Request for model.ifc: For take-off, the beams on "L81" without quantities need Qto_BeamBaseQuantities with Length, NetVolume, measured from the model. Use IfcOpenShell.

First a look at what the model holds.

```python
import ifcopenshell
import ifcopenshell.util.element
import ifcopenshell.util.unit

model = ifcopenshell.open("model.ifc")
print(model.schema)
for unit_type in ("LENGTHUNIT", "AREAUNIT", "VOLUMEUNIT"):
    print(unit_type, ifcopenshell.util.unit.calculate_unit_scale(model, unit_type))
storey = next(s for s in model.by_type("IfcBuildingStorey") if s.Name == "L81")
beams = [e for e in ifcopenshell.util.element.get_decomposition(storey) if e.is_a("IfcBeam")]
for e in sorted(beams, key=lambda e: e.id()):
    print(e.id(), e.is_a(), e.Name, list(ifcopenshell.util.element.get_psets(e, qtos_only=True)), sep=" | ")
```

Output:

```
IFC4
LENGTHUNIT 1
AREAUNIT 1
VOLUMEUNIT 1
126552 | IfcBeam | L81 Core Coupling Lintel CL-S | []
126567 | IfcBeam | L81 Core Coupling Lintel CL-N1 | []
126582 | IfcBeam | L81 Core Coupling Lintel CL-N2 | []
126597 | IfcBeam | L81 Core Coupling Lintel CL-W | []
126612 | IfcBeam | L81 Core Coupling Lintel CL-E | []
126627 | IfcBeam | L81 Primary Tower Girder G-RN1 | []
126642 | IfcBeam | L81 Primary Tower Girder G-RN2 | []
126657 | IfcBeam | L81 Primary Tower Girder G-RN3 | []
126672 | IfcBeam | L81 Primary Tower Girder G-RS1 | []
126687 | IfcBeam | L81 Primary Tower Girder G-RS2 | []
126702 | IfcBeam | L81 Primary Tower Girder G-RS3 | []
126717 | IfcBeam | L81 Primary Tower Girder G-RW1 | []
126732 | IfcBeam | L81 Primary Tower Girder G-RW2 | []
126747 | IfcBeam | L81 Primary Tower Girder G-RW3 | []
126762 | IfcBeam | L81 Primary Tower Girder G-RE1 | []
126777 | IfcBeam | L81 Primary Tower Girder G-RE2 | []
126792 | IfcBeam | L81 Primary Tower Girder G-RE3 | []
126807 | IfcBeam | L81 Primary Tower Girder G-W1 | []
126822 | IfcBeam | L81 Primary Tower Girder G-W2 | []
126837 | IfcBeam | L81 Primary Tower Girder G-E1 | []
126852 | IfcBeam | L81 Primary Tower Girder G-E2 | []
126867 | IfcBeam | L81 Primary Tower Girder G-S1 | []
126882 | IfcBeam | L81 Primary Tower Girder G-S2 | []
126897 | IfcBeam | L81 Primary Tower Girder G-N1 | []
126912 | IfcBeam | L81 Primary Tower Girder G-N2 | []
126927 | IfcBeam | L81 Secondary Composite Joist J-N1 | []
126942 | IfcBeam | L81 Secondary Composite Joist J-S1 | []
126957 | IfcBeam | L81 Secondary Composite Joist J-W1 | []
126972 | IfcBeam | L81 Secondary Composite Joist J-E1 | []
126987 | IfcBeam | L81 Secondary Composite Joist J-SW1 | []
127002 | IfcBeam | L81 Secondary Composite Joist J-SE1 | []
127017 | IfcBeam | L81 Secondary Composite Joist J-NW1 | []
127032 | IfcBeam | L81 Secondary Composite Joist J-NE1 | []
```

```python
import ifcopenshell
import ifcopenshell.api.pset
import ifcopenshell.geom
import ifcopenshell.util.element
import ifcopenshell.util.shape
import ifcopenshell.util.unit

model = ifcopenshell.open("model.ifc")
unit_scale = ifcopenshell.util.unit.calculate_unit_scale(model)
volume_scale = ifcopenshell.util.unit.calculate_unit_scale(model, "VOLUMEUNIT")
settings = ifcopenshell.geom.settings()

storey = next(s for s in model.by_type("IfcBuildingStorey") if s.Name == "L81")
beams = [e for e in ifcopenshell.util.element.get_decomposition(storey) if e.is_a("IfcBeam")]

for e in sorted(beams, key=lambda e: e.id()):
    if ifcopenshell.util.element.get_psets(e, qtos_only=True, should_inherit=False):
        continue
    # Geometry comes back in metres, in the element's own axes.
    shape = ifcopenshell.geom.create_shape(settings, e)
    values = {
        "Length": ifcopenshell.util.shape.get_max_xyz(shape.geometry) / unit_scale,
        "NetVolume": ifcopenshell.util.shape.get_volume(shape.geometry) / volume_scale,
    }
    qto = ifcopenshell.api.pset.add_qto(model, product=e, name="Qto_BeamBaseQuantities")
    ifcopenshell.api.pset.edit_qto(model, qto=qto, properties=values)
    print(e.id(), {k: round(v, 3) for k, v in values.items()})

model.write("model_v2.ifc")
```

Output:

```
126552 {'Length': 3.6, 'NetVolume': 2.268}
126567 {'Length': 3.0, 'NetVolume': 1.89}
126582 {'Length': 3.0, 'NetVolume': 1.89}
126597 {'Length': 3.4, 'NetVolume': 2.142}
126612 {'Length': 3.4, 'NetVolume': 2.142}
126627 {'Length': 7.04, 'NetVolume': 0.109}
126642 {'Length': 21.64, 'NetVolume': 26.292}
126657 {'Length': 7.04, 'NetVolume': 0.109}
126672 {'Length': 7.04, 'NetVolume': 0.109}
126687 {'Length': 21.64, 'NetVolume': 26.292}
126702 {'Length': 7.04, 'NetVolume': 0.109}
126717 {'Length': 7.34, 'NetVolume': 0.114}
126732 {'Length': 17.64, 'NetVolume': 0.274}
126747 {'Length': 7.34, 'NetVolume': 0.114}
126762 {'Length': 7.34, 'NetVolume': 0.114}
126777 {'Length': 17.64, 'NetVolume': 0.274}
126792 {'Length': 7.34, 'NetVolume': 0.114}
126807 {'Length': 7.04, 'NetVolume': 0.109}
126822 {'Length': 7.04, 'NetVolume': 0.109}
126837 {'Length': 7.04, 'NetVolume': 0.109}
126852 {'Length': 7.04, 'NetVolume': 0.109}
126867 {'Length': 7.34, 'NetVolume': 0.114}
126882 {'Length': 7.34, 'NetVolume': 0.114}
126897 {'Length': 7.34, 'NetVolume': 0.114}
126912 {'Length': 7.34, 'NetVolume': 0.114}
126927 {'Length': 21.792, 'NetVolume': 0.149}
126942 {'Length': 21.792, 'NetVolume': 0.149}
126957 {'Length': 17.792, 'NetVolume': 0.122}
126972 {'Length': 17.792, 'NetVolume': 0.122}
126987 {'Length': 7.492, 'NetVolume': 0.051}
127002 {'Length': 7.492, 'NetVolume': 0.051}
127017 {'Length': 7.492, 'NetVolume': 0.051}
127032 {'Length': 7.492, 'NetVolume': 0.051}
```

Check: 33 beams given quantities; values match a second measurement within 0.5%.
